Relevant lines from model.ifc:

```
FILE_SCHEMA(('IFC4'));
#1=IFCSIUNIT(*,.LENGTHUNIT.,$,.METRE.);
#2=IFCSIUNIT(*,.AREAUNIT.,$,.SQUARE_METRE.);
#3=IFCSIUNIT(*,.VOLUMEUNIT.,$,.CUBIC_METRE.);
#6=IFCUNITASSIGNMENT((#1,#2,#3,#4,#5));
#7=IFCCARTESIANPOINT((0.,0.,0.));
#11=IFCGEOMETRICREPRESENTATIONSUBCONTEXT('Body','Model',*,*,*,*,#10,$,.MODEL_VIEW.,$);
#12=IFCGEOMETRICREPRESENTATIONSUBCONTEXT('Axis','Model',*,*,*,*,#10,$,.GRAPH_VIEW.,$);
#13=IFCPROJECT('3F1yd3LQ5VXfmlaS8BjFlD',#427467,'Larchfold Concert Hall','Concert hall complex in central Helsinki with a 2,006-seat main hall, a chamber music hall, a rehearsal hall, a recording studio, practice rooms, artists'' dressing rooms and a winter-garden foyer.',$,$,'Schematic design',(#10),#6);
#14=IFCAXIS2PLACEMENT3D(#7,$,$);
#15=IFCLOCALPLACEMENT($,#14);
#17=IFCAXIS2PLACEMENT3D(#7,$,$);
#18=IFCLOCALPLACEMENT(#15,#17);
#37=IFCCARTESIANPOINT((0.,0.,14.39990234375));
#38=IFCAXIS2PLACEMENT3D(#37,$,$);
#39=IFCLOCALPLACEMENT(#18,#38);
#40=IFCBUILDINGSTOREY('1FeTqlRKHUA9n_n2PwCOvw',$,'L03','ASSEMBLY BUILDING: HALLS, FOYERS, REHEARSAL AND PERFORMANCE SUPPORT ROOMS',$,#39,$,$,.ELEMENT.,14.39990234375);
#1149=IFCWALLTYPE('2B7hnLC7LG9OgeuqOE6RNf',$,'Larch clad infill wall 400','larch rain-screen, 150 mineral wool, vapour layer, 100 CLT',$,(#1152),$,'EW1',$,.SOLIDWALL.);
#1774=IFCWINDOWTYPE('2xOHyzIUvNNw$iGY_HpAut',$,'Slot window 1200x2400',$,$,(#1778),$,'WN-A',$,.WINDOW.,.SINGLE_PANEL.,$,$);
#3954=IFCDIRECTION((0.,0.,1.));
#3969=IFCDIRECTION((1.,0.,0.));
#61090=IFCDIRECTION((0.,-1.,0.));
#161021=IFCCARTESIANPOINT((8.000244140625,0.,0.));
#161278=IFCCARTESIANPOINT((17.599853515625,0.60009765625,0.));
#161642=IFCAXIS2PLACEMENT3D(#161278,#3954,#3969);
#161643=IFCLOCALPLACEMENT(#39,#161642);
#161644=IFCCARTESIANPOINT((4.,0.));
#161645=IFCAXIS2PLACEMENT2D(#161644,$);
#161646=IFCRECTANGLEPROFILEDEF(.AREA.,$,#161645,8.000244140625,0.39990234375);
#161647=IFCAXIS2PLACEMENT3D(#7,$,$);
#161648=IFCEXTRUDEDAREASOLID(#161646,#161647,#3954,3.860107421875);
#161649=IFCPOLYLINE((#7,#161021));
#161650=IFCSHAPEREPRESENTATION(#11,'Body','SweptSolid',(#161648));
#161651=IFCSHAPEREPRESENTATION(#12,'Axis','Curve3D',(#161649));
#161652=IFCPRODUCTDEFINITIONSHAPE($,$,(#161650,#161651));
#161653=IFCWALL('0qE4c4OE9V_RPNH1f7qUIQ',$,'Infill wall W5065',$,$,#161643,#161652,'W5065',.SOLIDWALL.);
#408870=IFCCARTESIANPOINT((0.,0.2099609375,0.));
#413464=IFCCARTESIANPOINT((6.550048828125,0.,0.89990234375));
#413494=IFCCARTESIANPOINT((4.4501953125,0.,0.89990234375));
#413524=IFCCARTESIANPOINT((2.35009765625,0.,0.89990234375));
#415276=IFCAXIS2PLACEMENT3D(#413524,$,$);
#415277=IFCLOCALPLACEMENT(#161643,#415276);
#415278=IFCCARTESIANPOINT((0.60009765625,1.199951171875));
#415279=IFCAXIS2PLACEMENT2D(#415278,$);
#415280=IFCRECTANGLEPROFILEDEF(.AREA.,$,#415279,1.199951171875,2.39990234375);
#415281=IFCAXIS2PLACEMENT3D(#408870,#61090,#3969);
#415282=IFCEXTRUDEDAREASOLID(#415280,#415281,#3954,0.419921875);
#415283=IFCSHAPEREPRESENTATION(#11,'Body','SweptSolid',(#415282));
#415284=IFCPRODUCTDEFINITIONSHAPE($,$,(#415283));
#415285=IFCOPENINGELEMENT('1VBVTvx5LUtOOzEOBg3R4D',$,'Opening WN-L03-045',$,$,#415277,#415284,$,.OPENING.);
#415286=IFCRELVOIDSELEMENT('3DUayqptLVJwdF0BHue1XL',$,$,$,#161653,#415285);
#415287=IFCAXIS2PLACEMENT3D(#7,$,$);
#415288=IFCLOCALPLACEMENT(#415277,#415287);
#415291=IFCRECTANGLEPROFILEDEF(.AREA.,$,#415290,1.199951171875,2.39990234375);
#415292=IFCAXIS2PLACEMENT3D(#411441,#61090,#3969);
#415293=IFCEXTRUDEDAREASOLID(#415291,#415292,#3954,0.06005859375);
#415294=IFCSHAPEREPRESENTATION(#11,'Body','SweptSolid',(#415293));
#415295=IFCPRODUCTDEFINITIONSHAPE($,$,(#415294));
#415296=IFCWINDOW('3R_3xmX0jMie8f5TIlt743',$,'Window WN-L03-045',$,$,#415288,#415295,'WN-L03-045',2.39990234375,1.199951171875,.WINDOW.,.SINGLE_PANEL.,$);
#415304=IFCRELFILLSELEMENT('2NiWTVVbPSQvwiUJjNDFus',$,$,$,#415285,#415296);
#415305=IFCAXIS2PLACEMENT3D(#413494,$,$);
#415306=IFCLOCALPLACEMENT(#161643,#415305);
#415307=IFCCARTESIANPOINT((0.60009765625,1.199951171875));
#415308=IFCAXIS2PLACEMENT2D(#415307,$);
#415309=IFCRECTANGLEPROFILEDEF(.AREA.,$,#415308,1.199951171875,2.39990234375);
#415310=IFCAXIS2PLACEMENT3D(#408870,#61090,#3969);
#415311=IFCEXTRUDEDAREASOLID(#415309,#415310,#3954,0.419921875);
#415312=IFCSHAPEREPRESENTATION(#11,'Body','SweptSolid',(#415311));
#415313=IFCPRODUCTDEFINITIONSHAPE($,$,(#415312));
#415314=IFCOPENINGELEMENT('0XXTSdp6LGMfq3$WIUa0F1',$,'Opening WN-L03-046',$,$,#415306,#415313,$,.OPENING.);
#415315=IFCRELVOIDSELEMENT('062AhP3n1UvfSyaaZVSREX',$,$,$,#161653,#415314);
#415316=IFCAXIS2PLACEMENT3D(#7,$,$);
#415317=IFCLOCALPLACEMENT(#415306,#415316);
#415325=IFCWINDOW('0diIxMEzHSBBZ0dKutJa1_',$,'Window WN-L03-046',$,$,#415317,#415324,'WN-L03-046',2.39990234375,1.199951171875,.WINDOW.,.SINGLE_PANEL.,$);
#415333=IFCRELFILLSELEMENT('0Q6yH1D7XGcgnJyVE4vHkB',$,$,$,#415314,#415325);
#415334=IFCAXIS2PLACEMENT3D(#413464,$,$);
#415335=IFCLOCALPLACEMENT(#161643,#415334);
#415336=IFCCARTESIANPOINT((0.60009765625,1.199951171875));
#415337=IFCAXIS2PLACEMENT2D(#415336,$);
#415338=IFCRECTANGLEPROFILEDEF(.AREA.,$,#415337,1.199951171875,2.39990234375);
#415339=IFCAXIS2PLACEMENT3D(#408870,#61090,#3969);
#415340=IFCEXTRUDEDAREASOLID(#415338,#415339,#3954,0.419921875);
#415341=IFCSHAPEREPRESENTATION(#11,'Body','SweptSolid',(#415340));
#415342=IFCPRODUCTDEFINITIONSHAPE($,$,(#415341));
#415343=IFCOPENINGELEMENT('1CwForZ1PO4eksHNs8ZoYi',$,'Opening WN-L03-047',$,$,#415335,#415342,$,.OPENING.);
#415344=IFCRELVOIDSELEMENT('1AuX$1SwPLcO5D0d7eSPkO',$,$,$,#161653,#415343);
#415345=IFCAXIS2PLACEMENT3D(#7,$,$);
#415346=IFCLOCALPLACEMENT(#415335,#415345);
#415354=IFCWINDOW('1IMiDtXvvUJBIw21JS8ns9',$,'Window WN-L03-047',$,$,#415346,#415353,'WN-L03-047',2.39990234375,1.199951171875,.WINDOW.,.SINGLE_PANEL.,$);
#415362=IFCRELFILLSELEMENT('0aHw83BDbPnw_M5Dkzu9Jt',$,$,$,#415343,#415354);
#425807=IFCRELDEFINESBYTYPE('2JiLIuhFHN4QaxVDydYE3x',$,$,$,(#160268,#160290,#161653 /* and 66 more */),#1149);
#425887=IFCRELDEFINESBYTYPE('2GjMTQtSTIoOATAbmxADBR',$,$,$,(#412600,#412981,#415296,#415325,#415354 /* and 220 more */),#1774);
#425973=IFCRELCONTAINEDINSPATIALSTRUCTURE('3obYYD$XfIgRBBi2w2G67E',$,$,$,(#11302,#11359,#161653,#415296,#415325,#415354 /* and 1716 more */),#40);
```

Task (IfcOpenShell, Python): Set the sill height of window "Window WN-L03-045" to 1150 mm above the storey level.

```python
import numpy as np
import ifcopenshell
import ifcopenshell.api.geometry
import ifcopenshell.geom
import ifcopenshell.util.element
import ifcopenshell.util.placement
import ifcopenshell.util.shape
import ifcopenshell.util.unit

model = ifcopenshell.open("model.ifc")
unit_scale = ifcopenshell.util.unit.calculate_unit_scale(model)

window = model.by_guid("3R_3xmX0jMie8f5TIlt743")
opening = window.FillsVoids[0].RelatingOpeningElement
storey = ifcopenshell.util.element.get_container(window, ifc_class="IfcBuildingStorey")
level = ifcopenshell.util.placement.get_local_placement(storey.ObjectPlacement)[2, 3]

# The opening's origin need not be at the sill, so measure its lowest point.
shape = ifcopenshell.geom.create_shape(ifcopenshell.geom.settings(), opening)
bottom = ifcopenshell.util.shape.get_shape_bottom_elevation(shape, shape.geometry) / unit_scale
dz = level + 1.15 - bottom

shift = np.array([0.0, 0.0, dz])
# The window is placed relative to its opening, so it follows when the opening moves.
matrix = ifcopenshell.util.placement.get_local_placement(opening.ObjectPlacement)
matrix[:3, 3] += shift
ifcopenshell.api.geometry.edit_object_placement(
    model, product=opening, matrix=matrix, is_si=False, should_transform_children=True
)

print(f"moved by {dz * unit_scale:+.3f} m")

model.write("model_v2.ifc")
```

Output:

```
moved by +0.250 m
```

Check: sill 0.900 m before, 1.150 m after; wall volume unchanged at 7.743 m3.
